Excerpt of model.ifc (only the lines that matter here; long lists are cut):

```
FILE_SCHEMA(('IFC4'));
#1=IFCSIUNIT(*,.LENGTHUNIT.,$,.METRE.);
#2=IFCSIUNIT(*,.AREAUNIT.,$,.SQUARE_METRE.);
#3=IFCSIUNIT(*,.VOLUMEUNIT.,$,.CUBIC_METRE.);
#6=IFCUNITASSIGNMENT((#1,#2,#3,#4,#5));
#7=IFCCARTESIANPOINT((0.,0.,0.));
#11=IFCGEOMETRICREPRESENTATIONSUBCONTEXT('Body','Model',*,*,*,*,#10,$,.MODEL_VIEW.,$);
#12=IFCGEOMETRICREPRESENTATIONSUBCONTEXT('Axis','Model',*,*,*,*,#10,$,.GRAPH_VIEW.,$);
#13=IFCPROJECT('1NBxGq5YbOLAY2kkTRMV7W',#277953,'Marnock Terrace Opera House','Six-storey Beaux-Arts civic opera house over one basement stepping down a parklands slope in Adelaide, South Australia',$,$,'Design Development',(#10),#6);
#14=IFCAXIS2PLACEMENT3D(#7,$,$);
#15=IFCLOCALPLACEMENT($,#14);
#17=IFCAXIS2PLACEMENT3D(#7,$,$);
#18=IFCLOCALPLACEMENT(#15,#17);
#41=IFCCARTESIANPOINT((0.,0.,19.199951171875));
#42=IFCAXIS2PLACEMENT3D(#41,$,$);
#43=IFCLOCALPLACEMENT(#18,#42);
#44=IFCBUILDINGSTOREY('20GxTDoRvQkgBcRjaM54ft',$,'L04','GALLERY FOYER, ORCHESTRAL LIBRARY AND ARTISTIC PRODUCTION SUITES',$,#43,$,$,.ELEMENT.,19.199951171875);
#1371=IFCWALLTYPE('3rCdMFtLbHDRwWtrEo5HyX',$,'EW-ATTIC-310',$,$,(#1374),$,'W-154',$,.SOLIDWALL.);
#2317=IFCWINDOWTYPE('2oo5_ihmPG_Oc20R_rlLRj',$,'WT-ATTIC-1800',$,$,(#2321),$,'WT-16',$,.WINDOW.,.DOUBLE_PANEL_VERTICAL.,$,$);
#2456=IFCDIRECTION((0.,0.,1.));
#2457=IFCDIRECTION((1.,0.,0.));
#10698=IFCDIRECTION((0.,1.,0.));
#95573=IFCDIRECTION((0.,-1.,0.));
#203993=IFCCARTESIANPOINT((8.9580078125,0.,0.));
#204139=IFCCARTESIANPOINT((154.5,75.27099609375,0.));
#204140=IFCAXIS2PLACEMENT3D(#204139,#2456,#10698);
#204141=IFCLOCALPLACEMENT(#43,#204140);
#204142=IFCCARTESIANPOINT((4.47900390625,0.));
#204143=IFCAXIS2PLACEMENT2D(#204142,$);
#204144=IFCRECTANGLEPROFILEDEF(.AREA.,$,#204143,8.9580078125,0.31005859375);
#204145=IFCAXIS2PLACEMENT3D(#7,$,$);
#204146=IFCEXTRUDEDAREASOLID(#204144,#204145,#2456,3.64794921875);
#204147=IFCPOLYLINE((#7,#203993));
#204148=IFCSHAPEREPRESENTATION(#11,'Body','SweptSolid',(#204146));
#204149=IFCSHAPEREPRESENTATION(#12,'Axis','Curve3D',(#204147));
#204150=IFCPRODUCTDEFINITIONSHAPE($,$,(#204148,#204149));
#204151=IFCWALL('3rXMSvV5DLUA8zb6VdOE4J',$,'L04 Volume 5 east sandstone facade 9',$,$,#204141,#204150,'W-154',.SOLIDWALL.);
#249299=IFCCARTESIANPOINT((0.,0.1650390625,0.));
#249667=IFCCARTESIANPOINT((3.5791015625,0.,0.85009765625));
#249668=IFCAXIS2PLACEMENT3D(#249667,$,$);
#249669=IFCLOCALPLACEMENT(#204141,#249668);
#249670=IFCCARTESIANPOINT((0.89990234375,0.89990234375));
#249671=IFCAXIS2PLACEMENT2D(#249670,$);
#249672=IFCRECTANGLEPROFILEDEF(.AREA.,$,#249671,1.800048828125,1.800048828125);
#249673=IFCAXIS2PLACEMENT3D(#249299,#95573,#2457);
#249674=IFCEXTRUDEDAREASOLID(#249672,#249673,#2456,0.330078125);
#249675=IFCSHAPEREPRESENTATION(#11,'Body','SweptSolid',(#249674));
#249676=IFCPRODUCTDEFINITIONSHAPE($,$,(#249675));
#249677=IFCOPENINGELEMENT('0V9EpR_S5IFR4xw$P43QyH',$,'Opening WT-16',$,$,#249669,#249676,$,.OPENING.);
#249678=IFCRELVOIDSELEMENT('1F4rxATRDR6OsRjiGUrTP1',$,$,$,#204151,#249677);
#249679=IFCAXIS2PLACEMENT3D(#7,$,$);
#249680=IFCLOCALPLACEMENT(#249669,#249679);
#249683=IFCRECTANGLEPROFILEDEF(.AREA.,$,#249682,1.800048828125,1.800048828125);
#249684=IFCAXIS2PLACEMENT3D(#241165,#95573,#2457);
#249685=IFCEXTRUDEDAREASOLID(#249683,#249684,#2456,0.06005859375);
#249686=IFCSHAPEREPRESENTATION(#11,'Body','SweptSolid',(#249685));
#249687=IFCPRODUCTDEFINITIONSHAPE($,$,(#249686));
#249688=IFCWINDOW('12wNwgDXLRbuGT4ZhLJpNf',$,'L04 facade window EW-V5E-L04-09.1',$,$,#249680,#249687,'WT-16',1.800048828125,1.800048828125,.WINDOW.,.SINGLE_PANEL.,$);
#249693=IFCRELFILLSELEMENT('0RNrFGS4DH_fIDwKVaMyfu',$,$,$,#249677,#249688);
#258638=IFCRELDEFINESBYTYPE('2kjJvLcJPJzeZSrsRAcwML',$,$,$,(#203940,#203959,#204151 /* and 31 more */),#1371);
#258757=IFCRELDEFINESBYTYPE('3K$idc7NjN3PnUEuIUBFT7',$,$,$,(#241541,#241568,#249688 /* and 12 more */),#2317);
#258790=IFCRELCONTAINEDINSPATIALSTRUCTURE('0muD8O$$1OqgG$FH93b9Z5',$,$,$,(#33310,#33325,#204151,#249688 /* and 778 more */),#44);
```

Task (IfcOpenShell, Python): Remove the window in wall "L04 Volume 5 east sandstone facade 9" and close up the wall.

```python
import ifcopenshell
import ifcopenshell.api.feature
import ifcopenshell.api.root
import ifcopenshell.geom
import ifcopenshell.util.shape

model = ifcopenshell.open("model.ifc")
settings = ifcopenshell.geom.settings()


def volume(element):
    """Net volume in cubic metres, openings subtracted."""
    shape = ifcopenshell.geom.create_shape(settings, element)
    return ifcopenshell.util.shape.get_volume(shape.geometry)


window = model.by_id(249688)
opening = window.FillsVoids[0].RelatingOpeningElement
wall = opening.VoidsElements[0].RelatingBuildingElement
before = volume(wall)

ifcopenshell.api.root.remove_product(model, product=window)
ifcopenshell.api.feature.remove_feature(model, feature=opening)

after = volume(wall)

print(f"wall volume {before:.3f} -> {after:.3f} m3")

model.write("model_v2.ifc")
```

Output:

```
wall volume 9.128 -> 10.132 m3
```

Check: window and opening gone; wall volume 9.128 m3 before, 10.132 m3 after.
